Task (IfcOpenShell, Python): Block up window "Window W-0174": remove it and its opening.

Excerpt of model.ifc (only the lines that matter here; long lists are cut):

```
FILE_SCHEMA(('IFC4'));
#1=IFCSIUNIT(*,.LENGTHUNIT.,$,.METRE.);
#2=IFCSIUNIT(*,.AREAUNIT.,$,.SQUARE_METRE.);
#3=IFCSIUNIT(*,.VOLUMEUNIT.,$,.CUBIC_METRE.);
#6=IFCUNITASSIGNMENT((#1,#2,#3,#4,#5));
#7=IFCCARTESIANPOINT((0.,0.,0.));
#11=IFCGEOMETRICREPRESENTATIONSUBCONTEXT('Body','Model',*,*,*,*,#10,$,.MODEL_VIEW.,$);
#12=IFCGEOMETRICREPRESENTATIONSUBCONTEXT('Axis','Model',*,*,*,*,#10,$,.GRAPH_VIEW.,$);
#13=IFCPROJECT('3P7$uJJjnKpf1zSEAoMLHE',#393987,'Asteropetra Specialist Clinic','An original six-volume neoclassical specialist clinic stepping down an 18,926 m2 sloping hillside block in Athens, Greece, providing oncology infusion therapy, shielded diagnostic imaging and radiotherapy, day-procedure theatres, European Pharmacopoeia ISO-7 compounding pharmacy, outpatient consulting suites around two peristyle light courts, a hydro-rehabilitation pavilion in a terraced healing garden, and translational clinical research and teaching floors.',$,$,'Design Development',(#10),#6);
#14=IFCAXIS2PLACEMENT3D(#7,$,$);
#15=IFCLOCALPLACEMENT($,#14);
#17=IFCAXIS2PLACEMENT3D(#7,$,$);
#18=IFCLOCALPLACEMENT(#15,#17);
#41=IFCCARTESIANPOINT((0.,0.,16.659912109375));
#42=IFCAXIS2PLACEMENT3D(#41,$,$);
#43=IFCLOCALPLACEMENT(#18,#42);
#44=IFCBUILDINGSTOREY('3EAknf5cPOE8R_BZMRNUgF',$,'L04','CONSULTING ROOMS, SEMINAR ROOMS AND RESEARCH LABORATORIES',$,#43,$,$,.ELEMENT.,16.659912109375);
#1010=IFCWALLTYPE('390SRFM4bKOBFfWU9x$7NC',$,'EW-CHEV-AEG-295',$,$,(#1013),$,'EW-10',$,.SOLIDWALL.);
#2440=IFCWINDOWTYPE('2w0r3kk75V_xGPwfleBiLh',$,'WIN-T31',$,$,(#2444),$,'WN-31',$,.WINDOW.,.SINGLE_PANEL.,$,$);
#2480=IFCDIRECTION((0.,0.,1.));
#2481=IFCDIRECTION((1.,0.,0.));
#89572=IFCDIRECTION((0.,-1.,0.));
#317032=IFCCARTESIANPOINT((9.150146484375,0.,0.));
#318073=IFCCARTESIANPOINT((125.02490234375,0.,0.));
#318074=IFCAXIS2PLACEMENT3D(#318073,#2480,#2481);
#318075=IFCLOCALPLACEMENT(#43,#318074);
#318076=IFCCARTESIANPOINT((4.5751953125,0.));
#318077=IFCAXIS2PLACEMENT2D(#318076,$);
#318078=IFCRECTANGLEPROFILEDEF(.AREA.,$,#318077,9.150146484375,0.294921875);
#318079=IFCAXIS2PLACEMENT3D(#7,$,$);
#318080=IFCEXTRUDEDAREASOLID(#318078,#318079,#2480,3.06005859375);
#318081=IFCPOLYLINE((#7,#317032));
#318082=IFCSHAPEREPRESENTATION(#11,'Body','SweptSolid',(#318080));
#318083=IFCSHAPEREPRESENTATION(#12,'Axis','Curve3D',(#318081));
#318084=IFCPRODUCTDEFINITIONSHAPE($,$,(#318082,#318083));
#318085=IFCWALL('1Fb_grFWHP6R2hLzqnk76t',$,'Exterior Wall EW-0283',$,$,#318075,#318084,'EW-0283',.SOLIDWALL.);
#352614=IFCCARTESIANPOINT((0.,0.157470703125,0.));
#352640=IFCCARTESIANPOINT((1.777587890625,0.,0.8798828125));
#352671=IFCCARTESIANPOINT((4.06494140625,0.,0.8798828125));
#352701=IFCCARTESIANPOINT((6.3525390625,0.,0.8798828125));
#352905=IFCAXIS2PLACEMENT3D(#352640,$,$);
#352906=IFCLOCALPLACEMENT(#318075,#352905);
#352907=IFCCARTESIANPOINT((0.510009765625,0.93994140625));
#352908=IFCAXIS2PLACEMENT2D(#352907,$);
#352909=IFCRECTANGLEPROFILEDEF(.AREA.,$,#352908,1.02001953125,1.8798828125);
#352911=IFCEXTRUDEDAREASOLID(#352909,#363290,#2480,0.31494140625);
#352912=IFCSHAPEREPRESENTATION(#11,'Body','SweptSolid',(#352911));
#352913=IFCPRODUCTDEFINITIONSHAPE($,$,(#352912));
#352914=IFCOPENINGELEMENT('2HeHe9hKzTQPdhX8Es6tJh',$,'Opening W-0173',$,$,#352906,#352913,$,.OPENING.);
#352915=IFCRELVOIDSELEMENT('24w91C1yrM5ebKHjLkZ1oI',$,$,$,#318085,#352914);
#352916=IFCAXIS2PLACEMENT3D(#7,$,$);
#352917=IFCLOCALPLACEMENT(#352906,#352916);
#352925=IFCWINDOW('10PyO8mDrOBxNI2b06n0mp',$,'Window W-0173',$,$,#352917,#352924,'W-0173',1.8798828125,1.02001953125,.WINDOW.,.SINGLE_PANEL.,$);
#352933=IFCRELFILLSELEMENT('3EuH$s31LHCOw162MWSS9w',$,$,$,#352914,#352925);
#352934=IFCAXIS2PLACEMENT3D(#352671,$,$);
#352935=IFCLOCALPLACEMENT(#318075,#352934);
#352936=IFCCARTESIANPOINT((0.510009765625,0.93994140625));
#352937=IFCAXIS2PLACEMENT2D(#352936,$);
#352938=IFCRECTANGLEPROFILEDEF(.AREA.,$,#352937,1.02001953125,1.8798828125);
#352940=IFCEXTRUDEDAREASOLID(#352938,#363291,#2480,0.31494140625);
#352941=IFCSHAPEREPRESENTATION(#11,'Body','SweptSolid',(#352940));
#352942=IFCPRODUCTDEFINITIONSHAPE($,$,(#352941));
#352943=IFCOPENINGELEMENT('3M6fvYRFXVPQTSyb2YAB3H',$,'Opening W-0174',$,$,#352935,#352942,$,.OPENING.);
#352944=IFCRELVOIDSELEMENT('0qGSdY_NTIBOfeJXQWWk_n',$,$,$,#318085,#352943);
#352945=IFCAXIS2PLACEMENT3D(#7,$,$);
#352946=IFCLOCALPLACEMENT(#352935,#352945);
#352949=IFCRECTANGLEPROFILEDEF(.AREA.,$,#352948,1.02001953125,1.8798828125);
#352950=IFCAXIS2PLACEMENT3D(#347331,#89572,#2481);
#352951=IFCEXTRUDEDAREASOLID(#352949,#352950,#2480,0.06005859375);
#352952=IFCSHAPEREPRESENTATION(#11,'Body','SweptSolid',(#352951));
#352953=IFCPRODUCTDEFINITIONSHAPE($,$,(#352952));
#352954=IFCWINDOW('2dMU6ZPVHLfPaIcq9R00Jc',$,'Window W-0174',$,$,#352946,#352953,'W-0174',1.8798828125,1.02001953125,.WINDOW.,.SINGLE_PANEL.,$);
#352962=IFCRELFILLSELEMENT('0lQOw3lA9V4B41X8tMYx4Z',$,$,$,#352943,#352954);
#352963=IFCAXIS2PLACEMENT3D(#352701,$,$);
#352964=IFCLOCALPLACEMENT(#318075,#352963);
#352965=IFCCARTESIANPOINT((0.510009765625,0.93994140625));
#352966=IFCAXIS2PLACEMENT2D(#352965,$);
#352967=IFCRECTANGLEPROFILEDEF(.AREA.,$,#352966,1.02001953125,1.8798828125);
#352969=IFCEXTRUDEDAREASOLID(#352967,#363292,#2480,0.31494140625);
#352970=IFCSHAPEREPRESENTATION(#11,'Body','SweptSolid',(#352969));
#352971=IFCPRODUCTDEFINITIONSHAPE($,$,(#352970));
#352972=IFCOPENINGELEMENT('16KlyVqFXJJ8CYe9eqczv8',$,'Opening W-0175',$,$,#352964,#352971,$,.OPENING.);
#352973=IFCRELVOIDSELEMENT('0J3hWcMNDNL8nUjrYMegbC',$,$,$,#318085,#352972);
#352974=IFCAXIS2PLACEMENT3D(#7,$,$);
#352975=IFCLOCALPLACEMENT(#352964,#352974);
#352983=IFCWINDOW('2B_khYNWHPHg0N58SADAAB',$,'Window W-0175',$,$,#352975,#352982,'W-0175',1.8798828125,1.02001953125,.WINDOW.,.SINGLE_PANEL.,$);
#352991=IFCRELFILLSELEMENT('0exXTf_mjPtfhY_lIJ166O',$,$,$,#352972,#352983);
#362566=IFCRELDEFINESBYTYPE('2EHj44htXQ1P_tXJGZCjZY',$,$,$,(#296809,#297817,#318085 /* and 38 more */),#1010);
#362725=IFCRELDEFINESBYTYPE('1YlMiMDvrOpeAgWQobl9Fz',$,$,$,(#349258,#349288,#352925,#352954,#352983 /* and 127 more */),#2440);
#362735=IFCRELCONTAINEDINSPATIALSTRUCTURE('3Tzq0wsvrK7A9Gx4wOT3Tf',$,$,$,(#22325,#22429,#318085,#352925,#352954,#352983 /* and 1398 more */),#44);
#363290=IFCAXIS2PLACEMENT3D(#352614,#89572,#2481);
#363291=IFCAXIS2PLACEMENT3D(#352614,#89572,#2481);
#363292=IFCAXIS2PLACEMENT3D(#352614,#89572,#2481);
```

```python
import ifcopenshell
import ifcopenshell.api.feature
import ifcopenshell.api.root
import ifcopenshell.geom
import ifcopenshell.util.shape

model = ifcopenshell.open("model.ifc")
settings = ifcopenshell.geom.settings()


def volume(element):
    """Net volume in cubic metres, openings subtracted."""
    shape = ifcopenshell.geom.create_shape(settings, element)
    return ifcopenshell.util.shape.get_volume(shape.geometry)


window = model.by_guid("2dMU6ZPVHLfPaIcq9R00Jc")
opening = window.FillsVoids[0].RelatingOpeningElement
wall = opening.VoidsElements[0].RelatingBuildingElement
before = volume(wall)

ifcopenshell.api.root.remove_product(model, product=window)
ifcopenshell.api.feature.remove_feature(model, feature=opening)

after = volume(wall)

print(f"wall volume {before:.3f} -> {after:.3f} m3")

model.write("model_v2.ifc")
```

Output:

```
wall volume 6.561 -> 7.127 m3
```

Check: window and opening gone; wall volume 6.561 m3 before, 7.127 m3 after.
